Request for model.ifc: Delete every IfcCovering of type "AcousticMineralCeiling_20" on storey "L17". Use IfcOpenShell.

First a look at what the model holds.

```python
import ifcopenshell
import ifcopenshell.util.element

model = ifcopenshell.open("model.ifc")
print(model.schema)
storey = next(s for s in model.by_type("IfcBuildingStorey") if s.Name == "L17")
coverings = [e for e in ifcopenshell.util.element.get_decomposition(storey) if e.is_a("IfcCovering")]
seen = {}
for e in coverings:
    element_type = ifcopenshell.util.element.get_type(e)
    name = element_type.Name if element_type not in (None, e) else None
    seen[name] = seen.get(name, 0) + 1
for name, count in sorted(seen.items(), key=str):
    print(count, "x", name)
```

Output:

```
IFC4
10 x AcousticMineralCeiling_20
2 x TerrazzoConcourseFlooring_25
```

```python
import ifcopenshell
import ifcopenshell.api.root
import ifcopenshell.util.element

model = ifcopenshell.open("model.ifc")

storey = next(s for s in model.by_type("IfcBuildingStorey") if s.Name == "L17")
coverings = [e for e in ifcopenshell.util.element.get_decomposition(storey) if e.is_a("IfcCovering")]
targets = [e for e in coverings if (t := ifcopenshell.util.element.get_type(e)) not in (None, e) and t.Name == "AcousticMineralCeiling_20"]

for e in targets:
    ifcopenshell.api.root.remove_product(model, product=e)
print(len(targets), "removed")

model.write("model_edited.ifc")
```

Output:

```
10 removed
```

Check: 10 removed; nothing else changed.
